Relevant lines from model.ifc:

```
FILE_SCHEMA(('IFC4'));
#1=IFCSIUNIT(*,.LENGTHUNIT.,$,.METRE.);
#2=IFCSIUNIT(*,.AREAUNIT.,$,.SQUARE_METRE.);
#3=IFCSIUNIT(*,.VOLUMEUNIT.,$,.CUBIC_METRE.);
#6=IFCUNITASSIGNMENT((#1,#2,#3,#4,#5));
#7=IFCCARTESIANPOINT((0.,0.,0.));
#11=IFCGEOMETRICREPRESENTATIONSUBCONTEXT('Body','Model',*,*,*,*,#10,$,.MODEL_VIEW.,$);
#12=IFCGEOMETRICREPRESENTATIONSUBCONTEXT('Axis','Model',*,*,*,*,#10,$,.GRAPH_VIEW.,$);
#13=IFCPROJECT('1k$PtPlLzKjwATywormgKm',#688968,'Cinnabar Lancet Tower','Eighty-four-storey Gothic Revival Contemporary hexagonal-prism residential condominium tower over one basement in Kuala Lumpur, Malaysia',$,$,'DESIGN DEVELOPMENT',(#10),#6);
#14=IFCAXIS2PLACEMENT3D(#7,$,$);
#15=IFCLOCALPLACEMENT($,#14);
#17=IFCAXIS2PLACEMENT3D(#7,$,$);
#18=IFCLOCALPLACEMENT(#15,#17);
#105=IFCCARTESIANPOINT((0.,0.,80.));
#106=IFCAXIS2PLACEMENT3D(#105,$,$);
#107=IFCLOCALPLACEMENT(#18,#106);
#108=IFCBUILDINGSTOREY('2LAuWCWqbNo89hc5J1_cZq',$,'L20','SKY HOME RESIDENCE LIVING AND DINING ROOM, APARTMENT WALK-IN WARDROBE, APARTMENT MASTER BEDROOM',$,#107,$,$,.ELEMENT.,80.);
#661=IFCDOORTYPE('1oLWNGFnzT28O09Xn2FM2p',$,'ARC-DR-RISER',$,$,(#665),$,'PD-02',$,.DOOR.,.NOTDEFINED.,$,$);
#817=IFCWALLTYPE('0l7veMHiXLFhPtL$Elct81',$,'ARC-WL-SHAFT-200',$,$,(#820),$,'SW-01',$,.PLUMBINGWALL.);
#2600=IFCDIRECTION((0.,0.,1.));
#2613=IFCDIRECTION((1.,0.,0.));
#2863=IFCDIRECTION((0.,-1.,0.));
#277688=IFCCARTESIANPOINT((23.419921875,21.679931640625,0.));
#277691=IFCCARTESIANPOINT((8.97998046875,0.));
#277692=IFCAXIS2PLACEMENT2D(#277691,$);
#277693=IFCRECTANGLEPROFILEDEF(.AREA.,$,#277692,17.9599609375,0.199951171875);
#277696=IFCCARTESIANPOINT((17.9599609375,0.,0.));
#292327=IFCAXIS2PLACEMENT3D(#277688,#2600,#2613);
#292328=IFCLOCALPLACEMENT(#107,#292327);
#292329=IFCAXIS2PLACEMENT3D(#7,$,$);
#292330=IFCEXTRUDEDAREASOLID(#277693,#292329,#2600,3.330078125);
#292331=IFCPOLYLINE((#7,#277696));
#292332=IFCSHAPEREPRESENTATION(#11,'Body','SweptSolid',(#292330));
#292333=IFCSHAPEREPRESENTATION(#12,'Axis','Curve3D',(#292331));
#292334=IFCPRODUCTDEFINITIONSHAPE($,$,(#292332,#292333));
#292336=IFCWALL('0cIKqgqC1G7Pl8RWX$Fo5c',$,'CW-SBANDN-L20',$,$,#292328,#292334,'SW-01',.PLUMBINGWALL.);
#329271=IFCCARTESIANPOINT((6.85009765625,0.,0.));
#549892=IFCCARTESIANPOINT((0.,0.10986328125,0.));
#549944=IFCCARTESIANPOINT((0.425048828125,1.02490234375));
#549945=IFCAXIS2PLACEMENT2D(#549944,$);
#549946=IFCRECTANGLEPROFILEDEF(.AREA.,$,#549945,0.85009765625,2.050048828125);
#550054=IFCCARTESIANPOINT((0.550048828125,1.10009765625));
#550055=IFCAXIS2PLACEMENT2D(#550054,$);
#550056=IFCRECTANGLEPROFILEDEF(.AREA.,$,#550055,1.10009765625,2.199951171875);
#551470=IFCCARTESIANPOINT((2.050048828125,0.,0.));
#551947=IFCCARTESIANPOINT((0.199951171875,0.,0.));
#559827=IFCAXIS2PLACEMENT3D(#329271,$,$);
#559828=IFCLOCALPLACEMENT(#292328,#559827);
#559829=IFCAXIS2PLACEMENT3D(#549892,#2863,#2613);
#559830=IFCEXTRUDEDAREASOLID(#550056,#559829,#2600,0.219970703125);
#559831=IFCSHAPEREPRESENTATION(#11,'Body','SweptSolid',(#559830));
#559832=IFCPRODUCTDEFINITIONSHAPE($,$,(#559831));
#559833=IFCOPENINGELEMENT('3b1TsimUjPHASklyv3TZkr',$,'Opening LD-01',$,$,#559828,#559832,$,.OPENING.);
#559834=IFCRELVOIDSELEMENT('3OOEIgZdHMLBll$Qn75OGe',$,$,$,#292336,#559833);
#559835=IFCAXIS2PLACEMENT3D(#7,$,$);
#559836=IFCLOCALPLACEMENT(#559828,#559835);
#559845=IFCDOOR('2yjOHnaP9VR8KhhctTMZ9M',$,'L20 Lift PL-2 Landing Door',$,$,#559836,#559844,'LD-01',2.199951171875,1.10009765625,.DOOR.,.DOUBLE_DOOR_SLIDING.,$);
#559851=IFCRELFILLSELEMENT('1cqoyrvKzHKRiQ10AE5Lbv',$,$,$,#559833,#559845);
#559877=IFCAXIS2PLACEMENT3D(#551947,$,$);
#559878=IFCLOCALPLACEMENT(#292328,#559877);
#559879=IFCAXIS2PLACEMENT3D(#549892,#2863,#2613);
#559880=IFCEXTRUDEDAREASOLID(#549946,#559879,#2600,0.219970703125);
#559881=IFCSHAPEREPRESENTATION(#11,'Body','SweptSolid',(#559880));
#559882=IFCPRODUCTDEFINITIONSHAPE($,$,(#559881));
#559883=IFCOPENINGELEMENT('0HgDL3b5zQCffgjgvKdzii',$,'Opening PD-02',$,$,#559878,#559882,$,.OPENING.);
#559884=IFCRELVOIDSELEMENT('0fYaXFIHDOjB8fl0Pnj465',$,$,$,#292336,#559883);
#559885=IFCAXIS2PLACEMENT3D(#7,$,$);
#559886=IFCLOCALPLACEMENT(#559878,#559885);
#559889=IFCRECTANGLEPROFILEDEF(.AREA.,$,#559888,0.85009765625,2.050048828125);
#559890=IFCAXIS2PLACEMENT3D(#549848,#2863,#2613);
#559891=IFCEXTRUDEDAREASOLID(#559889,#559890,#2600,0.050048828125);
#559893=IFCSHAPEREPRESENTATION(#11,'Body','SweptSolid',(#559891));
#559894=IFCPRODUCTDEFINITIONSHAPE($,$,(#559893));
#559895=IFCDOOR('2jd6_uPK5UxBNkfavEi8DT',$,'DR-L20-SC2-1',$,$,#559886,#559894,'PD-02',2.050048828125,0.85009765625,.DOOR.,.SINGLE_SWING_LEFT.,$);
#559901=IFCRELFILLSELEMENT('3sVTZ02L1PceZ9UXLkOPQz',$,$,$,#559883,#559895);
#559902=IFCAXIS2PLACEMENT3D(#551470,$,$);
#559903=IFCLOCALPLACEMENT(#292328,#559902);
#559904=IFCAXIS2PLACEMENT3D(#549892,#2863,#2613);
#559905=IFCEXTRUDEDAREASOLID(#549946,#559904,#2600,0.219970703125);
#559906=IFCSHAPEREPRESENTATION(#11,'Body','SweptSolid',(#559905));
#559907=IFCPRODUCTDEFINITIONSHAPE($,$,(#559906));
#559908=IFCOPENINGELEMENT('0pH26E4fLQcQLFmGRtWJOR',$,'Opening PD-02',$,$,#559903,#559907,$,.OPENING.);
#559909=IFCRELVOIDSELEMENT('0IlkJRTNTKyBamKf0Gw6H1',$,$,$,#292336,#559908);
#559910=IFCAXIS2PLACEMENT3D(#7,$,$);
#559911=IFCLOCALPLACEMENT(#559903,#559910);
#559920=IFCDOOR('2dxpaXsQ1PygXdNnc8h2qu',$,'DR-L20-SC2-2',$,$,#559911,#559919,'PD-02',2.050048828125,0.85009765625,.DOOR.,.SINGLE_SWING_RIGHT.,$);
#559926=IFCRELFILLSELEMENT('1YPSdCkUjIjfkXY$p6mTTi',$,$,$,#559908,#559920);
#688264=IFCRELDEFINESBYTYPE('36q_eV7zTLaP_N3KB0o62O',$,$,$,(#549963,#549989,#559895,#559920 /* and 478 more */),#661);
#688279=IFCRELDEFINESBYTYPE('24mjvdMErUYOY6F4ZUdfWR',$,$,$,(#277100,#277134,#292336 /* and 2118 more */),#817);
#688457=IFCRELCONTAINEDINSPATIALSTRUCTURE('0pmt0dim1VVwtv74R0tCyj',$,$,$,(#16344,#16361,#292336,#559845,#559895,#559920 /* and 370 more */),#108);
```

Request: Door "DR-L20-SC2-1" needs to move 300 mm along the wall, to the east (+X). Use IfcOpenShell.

```python
import ifcopenshell
import ifcopenshell.api.geometry
import ifcopenshell.util.placement

model = ifcopenshell.open("model.ifc")

door = model.by_guid("2jd6_uPK5UxBNkfavEi8DT")
opening = door.FillsVoids[0].RelatingOpeningElement
wall = opening.VoidsElements[0].RelatingBuildingElement

wall_matrix = ifcopenshell.util.placement.get_local_placement(wall.ObjectPlacement)
shift = wall_matrix[:3, 0] * 0.3
before = ifcopenshell.util.placement.get_local_placement(door.ObjectPlacement)[:3, 3].copy()

# The door is placed relative to its opening, so it follows when the opening moves.
matrix = ifcopenshell.util.placement.get_local_placement(opening.ObjectPlacement)
matrix[:3, 3] += shift
ifcopenshell.api.geometry.edit_object_placement(
    model, product=opening, matrix=matrix, is_si=False, should_transform_children=True
)

after = ifcopenshell.util.placement.get_local_placement(door.ObjectPlacement)[:3, 3]
print("door moved by", (after - before).round(3) + 0.0)

model.write("model_edited.ifc")
```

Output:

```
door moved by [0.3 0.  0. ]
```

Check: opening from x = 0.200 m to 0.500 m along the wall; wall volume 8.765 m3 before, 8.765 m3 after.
